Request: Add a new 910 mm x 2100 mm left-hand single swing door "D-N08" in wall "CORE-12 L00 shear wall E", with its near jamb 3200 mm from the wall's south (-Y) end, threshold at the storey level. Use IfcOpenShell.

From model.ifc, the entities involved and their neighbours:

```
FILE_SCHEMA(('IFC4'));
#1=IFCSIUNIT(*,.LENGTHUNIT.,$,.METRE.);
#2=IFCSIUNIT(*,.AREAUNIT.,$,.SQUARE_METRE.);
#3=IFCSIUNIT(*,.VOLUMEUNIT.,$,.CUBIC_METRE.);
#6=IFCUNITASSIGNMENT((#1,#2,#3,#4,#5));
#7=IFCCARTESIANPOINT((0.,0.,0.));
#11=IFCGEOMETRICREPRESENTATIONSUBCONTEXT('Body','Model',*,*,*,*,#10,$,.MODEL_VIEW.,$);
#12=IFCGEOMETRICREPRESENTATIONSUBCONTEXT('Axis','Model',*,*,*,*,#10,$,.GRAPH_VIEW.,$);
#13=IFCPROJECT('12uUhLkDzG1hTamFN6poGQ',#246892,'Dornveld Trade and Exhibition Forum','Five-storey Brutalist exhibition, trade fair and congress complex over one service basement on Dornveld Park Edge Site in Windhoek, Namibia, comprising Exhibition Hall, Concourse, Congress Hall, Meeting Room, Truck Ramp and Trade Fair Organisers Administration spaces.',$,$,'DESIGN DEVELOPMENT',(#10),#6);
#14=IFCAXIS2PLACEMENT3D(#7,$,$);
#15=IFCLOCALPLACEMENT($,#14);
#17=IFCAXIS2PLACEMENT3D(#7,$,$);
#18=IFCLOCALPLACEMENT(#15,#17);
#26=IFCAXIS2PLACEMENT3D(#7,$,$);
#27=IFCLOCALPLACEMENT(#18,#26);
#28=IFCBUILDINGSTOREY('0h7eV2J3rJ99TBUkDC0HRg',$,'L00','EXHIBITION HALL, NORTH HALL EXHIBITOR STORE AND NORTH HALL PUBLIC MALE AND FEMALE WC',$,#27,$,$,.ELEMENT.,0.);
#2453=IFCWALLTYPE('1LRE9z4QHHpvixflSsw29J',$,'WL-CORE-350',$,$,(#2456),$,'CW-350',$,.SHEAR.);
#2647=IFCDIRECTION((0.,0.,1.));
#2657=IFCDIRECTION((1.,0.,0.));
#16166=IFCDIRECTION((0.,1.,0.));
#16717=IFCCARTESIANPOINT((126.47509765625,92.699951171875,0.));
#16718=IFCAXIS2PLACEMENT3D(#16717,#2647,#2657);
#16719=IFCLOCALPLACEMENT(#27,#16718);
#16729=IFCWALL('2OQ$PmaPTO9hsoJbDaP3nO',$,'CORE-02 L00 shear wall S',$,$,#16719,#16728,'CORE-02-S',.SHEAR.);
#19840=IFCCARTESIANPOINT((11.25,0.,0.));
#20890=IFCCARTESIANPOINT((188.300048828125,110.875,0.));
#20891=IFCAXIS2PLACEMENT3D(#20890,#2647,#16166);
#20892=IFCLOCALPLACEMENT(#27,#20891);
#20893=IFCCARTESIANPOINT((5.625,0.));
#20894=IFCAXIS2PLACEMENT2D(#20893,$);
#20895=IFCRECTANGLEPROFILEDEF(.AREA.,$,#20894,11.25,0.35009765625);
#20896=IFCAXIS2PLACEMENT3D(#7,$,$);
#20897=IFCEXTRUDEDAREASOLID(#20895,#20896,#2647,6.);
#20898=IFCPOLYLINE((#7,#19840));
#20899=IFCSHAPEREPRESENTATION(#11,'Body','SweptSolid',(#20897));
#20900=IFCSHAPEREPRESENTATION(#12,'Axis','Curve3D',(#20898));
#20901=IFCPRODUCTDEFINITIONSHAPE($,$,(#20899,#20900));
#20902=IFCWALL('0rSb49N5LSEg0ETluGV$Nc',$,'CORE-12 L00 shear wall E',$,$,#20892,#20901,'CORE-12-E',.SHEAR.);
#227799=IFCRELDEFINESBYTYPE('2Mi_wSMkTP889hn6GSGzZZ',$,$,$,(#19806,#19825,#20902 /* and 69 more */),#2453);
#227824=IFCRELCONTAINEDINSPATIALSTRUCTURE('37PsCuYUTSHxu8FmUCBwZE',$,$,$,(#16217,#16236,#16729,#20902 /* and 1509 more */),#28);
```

```python
import numpy as np
import ifcopenshell
import ifcopenshell.api.feature
import ifcopenshell.api.geometry
import ifcopenshell.api.root
import ifcopenshell.api.spatial
import ifcopenshell.geom
import ifcopenshell.util.element
import ifcopenshell.util.placement
import ifcopenshell.util.representation
import ifcopenshell.util.shape
import ifcopenshell.util.unit

model = ifcopenshell.open("model.ifc")
unit_scale = ifcopenshell.util.unit.calculate_unit_scale(model)
settings = ifcopenshell.geom.settings()


def volume(element):
    """Net volume in cubic metres, openings subtracted."""
    shape = ifcopenshell.geom.create_shape(settings, element)
    return ifcopenshell.util.shape.get_volume(shape.geometry)


wall = model.by_guid("0rSb49N5LSEg0ETluGV$Nc")
storey = ifcopenshell.util.element.get_container(wall, ifc_class="IfcBuildingStorey")
context = ifcopenshell.util.representation.get_context(model, "Model", "Body", "MODEL_VIEW")
before = volume(wall)

width, height, from_end, sill = 0.91, 2.1, 3.2, 0.0  # metres

# The wall runs along its own X axis, and the end named is its -X end.
wall_shape = ifcopenshell.geom.create_shape(settings, wall)
x, y, z = ifcopenshell.util.shape.get_vertices(wall_shape.geometry).T
start = x.min() + from_end
face, thickness = float(y.min()), float(y.max() - y.min())
wall_matrix = ifcopenshell.util.placement.get_local_placement(wall.ObjectPlacement)
level = ifcopenshell.util.placement.get_local_placement(storey.ObjectPlacement)[2, 3]


def in_wall(x, y):
    """Placement at x, y metres in the wall's axes, at sill height."""
    matrix = wall_matrix.copy()
    matrix[:, 3] = wall_matrix @ np.array([x / unit_scale, y / unit_scale, 0.0, 1.0])
    matrix[2, 3] = level + sill / unit_scale
    return matrix


# Opening: a box that overshoots both wall faces by 50 mm.
opening = ifcopenshell.api.root.create_entity(model, ifc_class="IfcOpeningElement", predefined_type="OPENING")
box = ifcopenshell.api.geometry.add_wall_representation(
    model, context=context, length=width, height=height, thickness=thickness + 0.1
)
ifcopenshell.api.geometry.assign_representation(model, product=opening, representation=box)
ifcopenshell.api.geometry.edit_object_placement(model, product=opening, matrix=in_wall(start, face - 0.05), is_si=False)
ifcopenshell.api.feature.add_feature(model, feature=opening, element=wall)

door = ifcopenshell.api.root.create_entity(model, ifc_class="IfcDoor", name="D-N08", predefined_type="DOOR")
door.OverallWidth, door.OverallHeight = width / unit_scale, height / unit_scale
door.OperationType = "SINGLE_SWING_LEFT"
body = ifcopenshell.api.geometry.add_door_representation(
    model,
    context=context,
    overall_width=door.OverallWidth,
    overall_height=door.OverallHeight,
    operation_type="SINGLE_SWING_LEFT",
    lining_properties={"LiningDepth": thickness / unit_scale, "ThresholdDepth": thickness / unit_scale},
)
ifcopenshell.api.geometry.assign_representation(model, product=door, representation=body)
ifcopenshell.api.spatial.assign_container(model, products=[door], relating_structure=storey)
ifcopenshell.api.feature.add_filling(model, opening=opening, element=door)

# The lining spans the wall, so the door starts at the wall face.
ifcopenshell.api.geometry.edit_object_placement(model, product=door, matrix=in_wall(start, face), is_si=False)

after = volume(wall)

print(f"wall volume {before:.3f} -> {after:.3f} m3")

model.write("model-out.ifc")
```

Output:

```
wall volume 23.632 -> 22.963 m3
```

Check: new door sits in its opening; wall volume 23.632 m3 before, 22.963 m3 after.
